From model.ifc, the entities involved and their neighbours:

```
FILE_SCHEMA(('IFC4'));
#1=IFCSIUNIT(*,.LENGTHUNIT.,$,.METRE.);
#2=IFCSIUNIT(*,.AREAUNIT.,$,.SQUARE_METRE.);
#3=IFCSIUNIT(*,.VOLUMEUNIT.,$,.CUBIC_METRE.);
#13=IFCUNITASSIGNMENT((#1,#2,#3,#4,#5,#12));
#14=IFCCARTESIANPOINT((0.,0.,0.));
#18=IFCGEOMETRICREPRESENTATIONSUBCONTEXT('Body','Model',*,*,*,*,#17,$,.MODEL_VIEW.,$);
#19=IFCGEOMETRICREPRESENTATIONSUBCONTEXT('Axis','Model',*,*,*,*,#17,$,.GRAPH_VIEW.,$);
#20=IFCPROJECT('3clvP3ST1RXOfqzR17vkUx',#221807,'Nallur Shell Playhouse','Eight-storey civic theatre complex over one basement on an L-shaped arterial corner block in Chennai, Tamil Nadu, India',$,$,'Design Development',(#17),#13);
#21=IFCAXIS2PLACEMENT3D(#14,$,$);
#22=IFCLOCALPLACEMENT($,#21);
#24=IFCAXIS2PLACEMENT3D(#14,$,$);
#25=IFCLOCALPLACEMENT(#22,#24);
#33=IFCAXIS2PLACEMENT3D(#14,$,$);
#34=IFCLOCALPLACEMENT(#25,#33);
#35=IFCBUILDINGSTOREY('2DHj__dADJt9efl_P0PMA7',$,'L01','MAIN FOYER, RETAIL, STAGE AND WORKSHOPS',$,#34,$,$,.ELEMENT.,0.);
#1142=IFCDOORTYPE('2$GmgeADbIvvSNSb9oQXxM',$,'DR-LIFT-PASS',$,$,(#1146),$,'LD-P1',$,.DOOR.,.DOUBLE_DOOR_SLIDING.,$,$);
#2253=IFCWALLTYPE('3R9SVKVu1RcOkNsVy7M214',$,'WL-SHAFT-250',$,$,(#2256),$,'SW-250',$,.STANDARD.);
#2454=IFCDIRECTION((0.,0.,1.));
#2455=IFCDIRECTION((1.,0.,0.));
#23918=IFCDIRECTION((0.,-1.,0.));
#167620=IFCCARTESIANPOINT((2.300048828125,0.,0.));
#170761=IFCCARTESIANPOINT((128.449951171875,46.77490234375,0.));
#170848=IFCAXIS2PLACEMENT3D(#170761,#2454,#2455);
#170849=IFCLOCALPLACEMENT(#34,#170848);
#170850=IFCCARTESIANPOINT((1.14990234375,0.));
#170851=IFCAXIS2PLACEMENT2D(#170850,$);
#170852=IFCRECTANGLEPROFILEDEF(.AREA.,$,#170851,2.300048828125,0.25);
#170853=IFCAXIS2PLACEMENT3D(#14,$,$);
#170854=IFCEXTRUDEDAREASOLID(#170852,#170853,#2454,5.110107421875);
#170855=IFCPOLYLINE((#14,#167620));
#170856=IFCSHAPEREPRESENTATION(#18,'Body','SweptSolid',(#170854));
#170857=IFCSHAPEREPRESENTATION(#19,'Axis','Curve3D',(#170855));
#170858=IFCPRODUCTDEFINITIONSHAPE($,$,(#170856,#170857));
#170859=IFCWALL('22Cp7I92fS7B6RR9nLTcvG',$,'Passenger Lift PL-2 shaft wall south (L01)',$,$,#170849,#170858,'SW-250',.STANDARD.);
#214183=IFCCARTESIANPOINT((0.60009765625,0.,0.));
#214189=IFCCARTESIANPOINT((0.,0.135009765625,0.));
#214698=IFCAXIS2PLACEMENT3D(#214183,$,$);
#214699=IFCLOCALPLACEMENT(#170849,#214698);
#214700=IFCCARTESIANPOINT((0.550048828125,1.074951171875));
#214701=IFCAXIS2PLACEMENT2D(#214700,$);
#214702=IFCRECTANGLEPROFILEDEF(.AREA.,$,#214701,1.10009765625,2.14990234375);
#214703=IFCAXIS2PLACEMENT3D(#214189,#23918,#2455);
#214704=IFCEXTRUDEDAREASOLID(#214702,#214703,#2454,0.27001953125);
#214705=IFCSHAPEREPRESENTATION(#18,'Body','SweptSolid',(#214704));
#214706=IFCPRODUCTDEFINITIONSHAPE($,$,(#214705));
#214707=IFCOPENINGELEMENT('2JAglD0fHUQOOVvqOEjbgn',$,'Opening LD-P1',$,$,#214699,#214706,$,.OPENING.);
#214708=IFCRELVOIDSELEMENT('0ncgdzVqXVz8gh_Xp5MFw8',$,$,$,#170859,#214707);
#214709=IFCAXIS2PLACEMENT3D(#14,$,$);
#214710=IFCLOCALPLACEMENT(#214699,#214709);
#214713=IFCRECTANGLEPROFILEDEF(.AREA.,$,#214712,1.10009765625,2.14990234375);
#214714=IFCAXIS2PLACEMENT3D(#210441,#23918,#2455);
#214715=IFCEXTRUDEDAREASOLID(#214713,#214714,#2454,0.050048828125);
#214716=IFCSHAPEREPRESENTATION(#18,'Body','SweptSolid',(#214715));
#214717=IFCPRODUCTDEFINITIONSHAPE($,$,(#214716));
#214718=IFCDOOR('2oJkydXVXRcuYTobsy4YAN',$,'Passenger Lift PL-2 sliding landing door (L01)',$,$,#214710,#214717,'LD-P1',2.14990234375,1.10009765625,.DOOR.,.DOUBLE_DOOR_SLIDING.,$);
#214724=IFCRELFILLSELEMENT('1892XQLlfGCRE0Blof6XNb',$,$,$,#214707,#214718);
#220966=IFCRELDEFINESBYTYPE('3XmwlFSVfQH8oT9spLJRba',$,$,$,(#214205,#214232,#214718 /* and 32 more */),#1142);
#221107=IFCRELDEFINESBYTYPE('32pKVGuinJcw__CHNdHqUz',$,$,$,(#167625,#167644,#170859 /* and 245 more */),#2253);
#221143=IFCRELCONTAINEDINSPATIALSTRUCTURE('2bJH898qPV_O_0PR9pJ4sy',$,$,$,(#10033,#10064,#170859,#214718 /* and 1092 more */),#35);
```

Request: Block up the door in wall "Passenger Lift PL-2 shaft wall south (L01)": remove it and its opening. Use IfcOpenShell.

```python
import ifcopenshell
import ifcopenshell.api.feature
import ifcopenshell.api.root
import ifcopenshell.geom
import ifcopenshell.util.shape

model = ifcopenshell.open("model.ifc")
settings = ifcopenshell.geom.settings()


def volume(element):
    """Net volume in cubic metres, openings subtracted."""
    shape = ifcopenshell.geom.create_shape(settings, element)
    return ifcopenshell.util.shape.get_volume(shape.geometry)


door = model.by_id(214718)
opening = door.FillsVoids[0].RelatingOpeningElement
wall = opening.VoidsElements[0].RelatingBuildingElement
before = volume(wall)

ifcopenshell.api.root.remove_product(model, product=door)
ifcopenshell.api.feature.remove_feature(model, feature=opening)

after = volume(wall)

print(f"wall volume {before:.3f} -> {after:.3f} m3")

model.write("model-out.ifc")
```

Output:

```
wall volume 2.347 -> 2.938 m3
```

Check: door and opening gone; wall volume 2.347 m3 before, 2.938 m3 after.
